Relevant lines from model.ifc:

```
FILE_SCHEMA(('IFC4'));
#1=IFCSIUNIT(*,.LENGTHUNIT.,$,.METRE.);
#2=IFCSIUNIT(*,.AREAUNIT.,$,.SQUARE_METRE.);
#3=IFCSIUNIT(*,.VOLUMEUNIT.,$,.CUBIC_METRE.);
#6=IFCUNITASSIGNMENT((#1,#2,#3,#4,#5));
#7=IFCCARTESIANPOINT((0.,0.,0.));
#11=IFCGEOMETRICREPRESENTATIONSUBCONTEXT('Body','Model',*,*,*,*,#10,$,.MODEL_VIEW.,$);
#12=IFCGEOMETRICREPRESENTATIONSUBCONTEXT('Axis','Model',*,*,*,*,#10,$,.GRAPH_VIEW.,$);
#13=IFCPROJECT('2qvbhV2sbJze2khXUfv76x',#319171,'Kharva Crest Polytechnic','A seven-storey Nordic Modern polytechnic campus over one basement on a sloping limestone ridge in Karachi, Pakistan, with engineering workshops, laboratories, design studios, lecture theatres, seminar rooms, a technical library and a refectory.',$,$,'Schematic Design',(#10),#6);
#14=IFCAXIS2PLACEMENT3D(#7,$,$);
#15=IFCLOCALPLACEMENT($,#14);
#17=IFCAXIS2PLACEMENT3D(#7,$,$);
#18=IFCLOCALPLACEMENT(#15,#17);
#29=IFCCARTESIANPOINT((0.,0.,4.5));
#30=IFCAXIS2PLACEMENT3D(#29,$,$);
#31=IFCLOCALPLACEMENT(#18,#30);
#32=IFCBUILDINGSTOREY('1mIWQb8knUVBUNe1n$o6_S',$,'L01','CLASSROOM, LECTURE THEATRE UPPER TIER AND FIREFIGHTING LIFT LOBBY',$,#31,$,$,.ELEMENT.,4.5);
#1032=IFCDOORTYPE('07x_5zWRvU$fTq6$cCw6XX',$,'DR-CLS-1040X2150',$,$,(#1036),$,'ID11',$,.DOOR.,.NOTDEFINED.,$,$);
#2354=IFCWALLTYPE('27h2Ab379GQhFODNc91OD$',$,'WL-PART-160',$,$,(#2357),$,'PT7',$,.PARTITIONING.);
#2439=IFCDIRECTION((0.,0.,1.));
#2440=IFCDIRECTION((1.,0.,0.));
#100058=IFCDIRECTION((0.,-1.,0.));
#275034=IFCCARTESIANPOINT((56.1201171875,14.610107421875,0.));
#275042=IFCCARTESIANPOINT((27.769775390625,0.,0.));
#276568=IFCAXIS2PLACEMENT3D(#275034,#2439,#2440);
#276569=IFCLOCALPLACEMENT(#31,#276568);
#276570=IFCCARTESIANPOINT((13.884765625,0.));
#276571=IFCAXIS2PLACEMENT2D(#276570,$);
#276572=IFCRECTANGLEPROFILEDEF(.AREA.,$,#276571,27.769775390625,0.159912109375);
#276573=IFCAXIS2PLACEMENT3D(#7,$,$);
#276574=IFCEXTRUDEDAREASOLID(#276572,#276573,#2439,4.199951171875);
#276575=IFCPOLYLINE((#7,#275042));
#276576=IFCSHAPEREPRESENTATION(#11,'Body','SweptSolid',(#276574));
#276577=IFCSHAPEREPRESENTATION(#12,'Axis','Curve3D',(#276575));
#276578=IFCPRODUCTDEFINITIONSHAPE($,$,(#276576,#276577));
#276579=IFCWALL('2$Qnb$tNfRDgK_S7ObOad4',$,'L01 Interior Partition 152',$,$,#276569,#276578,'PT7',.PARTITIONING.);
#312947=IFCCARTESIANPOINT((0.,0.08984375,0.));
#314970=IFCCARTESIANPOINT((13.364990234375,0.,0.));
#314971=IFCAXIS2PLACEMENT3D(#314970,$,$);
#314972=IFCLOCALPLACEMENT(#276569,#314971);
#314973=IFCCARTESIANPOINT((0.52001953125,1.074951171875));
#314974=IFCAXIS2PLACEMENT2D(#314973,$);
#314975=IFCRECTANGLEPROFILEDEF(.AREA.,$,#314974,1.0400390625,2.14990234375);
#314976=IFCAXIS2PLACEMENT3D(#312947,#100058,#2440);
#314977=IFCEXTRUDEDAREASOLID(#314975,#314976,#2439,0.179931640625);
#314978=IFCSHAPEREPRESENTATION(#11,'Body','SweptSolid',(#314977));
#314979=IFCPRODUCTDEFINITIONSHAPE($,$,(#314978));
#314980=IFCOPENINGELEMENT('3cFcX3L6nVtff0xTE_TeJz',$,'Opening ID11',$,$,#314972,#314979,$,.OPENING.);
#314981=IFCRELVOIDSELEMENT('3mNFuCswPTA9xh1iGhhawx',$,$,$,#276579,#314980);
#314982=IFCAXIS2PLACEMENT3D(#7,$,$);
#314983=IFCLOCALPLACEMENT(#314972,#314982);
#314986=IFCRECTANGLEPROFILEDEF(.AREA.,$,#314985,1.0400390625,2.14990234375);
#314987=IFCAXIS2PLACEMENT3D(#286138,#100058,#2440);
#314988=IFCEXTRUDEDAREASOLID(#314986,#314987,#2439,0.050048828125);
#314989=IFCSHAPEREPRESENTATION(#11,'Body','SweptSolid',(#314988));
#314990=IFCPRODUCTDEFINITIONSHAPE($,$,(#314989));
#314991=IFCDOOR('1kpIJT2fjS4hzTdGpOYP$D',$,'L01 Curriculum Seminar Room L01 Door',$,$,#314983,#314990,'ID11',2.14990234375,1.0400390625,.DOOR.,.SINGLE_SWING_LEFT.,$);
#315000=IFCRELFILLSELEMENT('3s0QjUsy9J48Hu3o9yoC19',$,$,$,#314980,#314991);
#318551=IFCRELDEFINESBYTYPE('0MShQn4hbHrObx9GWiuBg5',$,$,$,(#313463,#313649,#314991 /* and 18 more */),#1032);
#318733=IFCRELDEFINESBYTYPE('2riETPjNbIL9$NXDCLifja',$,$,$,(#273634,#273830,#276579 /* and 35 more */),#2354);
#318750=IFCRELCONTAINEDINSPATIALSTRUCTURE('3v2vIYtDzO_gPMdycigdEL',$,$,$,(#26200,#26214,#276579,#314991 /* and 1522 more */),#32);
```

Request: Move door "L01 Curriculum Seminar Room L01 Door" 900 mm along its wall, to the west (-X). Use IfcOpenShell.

```python
import ifcopenshell
import ifcopenshell.api.geometry
import ifcopenshell.util.placement
import ifcopenshell.util.unit

model = ifcopenshell.open("model.ifc")
unit_scale = ifcopenshell.util.unit.calculate_unit_scale(model)

door = model.by_guid("1kpIJT2fjS4hzTdGpOYP$D")
opening = door.FillsVoids[0].RelatingOpeningElement
wall = opening.VoidsElements[0].RelatingBuildingElement

wall_matrix = ifcopenshell.util.placement.get_local_placement(wall.ObjectPlacement)
shift = wall_matrix[:3, 0] * -0.9 / unit_scale
before = ifcopenshell.util.placement.get_local_placement(door.ObjectPlacement)[:3, 3].copy()

# The door is placed relative to its opening, so it follows when the opening moves.
matrix = ifcopenshell.util.placement.get_local_placement(opening.ObjectPlacement)
matrix[:3, 3] += shift
ifcopenshell.api.geometry.edit_object_placement(
    model, product=opening, matrix=matrix, is_si=False, should_transform_children=True
)

after = ifcopenshell.util.placement.get_local_placement(door.ObjectPlacement)[:3, 3]
print("door moved by", (after - before).round(3) + 0.0)

model.write("model_updated.ifc")
```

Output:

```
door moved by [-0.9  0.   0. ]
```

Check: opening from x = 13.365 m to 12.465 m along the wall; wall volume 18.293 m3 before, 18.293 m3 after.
